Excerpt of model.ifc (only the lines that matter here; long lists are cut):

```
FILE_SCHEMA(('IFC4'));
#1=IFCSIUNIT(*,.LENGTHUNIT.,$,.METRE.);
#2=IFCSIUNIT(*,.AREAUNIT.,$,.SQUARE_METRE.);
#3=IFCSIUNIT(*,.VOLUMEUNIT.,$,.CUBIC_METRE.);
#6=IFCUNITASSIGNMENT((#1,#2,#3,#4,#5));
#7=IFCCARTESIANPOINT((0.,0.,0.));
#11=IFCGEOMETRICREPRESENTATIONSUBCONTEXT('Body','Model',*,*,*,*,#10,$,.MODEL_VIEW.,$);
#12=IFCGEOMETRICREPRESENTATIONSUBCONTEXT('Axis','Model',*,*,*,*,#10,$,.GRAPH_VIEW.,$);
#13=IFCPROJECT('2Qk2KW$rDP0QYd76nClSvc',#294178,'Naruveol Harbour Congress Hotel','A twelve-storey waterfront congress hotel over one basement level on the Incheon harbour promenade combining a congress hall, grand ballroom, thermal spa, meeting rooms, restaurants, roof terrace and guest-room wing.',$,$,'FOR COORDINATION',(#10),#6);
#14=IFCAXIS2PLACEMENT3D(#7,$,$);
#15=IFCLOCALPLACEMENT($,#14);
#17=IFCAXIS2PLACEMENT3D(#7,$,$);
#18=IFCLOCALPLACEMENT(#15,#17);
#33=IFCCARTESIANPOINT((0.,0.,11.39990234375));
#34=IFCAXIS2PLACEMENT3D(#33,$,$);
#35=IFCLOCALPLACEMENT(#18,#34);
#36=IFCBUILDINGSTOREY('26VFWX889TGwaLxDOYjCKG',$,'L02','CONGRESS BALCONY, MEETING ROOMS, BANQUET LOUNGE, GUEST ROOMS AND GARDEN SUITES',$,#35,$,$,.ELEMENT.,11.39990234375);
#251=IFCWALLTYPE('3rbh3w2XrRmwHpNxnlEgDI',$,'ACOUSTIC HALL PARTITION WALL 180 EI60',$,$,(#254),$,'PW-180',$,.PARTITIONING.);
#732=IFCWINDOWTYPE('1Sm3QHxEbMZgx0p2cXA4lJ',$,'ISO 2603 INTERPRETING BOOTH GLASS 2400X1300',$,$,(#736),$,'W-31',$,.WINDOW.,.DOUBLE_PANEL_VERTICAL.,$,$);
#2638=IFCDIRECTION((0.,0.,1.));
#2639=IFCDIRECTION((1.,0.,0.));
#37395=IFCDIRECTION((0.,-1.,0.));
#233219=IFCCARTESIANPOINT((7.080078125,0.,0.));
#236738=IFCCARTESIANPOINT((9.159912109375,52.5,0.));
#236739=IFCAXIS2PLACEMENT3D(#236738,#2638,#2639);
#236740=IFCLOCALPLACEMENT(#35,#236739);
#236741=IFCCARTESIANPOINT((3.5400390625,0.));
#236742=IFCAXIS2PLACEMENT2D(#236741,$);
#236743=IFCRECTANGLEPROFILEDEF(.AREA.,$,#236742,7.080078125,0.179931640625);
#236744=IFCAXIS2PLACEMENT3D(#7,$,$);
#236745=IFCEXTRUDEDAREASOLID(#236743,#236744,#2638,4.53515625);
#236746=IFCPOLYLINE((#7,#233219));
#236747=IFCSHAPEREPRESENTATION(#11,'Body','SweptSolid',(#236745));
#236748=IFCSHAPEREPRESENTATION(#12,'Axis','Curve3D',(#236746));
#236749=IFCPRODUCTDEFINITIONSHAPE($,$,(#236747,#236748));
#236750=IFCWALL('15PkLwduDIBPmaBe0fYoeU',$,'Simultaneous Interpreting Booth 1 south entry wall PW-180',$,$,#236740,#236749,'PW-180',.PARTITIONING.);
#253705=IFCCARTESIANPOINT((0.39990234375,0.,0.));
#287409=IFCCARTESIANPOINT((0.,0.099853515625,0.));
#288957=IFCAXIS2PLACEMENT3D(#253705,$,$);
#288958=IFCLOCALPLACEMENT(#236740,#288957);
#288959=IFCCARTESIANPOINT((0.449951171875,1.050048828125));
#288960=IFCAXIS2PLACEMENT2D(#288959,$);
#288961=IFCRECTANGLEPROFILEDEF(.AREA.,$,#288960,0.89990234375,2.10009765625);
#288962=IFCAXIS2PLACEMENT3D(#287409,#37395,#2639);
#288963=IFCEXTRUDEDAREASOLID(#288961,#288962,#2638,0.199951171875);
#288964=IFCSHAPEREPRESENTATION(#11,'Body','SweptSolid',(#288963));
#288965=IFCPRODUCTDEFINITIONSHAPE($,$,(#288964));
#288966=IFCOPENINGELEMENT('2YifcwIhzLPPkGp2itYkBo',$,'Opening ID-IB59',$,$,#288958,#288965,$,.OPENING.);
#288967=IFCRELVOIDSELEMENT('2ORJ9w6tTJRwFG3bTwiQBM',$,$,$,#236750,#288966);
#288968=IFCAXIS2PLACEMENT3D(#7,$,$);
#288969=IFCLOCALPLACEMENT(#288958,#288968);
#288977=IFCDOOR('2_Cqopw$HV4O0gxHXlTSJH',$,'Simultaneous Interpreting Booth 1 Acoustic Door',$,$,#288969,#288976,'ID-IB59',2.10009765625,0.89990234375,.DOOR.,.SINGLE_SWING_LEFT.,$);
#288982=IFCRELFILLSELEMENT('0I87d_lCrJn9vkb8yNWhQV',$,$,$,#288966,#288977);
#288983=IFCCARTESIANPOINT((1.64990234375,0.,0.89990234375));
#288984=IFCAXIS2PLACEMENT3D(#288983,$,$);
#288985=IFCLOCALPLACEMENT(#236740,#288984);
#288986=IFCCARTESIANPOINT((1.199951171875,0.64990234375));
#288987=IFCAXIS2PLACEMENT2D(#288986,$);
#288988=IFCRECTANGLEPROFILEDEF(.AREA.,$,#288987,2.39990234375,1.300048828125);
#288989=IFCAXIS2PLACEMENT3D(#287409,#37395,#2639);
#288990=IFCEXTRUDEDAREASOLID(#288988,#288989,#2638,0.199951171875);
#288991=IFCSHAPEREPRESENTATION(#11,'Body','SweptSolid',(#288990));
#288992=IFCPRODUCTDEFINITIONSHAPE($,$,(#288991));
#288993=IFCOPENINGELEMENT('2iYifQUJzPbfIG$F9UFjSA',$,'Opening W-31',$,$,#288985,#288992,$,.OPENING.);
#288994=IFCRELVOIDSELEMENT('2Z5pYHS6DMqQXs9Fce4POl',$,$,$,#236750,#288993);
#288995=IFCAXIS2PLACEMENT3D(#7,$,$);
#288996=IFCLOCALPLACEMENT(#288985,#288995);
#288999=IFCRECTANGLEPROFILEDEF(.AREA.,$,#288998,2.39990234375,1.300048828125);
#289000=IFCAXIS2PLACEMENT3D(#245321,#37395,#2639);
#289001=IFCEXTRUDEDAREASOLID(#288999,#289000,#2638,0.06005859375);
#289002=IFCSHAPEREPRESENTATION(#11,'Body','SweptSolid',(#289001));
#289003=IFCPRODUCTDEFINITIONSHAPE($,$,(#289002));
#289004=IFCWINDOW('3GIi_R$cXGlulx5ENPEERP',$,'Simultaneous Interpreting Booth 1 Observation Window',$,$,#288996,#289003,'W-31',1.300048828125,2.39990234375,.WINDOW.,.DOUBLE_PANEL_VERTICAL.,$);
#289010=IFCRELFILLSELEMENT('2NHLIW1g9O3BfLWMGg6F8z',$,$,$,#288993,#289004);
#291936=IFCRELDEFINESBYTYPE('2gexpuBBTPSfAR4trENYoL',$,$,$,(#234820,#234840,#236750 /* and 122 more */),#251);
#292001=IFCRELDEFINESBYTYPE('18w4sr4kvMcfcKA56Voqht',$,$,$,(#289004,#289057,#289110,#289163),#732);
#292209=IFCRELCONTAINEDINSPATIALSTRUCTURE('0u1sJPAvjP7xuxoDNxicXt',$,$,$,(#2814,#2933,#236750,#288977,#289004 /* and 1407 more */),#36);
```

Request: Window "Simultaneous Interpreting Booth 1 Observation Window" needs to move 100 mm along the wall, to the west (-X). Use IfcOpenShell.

```python
import ifcopenshell
import ifcopenshell.api.geometry
import ifcopenshell.util.placement
import ifcopenshell.util.unit

model = ifcopenshell.open("model.ifc")
unit_scale = ifcopenshell.util.unit.calculate_unit_scale(model)

window = model.by_guid("3GIi_R$cXGlulx5ENPEERP")
opening = window.FillsVoids[0].RelatingOpeningElement
wall = opening.VoidsElements[0].RelatingBuildingElement

wall_matrix = ifcopenshell.util.placement.get_local_placement(wall.ObjectPlacement)
shift = wall_matrix[:3, 0] * -0.1 / unit_scale
before = ifcopenshell.util.placement.get_local_placement(window.ObjectPlacement)[:3, 3].copy()

# The window is placed relative to its opening, so it follows when the opening moves.
matrix = ifcopenshell.util.placement.get_local_placement(opening.ObjectPlacement)
matrix[:3, 3] += shift
ifcopenshell.api.geometry.edit_object_placement(
    model, product=opening, matrix=matrix, is_si=False, should_transform_children=True
)

after = ifcopenshell.util.placement.get_local_placement(window.ObjectPlacement)[:3, 3]
print("window moved by", (after - before).round(3) + 0.0)

model.write("model_edited.ifc")
```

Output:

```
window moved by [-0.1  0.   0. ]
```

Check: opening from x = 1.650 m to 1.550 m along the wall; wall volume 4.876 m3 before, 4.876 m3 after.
